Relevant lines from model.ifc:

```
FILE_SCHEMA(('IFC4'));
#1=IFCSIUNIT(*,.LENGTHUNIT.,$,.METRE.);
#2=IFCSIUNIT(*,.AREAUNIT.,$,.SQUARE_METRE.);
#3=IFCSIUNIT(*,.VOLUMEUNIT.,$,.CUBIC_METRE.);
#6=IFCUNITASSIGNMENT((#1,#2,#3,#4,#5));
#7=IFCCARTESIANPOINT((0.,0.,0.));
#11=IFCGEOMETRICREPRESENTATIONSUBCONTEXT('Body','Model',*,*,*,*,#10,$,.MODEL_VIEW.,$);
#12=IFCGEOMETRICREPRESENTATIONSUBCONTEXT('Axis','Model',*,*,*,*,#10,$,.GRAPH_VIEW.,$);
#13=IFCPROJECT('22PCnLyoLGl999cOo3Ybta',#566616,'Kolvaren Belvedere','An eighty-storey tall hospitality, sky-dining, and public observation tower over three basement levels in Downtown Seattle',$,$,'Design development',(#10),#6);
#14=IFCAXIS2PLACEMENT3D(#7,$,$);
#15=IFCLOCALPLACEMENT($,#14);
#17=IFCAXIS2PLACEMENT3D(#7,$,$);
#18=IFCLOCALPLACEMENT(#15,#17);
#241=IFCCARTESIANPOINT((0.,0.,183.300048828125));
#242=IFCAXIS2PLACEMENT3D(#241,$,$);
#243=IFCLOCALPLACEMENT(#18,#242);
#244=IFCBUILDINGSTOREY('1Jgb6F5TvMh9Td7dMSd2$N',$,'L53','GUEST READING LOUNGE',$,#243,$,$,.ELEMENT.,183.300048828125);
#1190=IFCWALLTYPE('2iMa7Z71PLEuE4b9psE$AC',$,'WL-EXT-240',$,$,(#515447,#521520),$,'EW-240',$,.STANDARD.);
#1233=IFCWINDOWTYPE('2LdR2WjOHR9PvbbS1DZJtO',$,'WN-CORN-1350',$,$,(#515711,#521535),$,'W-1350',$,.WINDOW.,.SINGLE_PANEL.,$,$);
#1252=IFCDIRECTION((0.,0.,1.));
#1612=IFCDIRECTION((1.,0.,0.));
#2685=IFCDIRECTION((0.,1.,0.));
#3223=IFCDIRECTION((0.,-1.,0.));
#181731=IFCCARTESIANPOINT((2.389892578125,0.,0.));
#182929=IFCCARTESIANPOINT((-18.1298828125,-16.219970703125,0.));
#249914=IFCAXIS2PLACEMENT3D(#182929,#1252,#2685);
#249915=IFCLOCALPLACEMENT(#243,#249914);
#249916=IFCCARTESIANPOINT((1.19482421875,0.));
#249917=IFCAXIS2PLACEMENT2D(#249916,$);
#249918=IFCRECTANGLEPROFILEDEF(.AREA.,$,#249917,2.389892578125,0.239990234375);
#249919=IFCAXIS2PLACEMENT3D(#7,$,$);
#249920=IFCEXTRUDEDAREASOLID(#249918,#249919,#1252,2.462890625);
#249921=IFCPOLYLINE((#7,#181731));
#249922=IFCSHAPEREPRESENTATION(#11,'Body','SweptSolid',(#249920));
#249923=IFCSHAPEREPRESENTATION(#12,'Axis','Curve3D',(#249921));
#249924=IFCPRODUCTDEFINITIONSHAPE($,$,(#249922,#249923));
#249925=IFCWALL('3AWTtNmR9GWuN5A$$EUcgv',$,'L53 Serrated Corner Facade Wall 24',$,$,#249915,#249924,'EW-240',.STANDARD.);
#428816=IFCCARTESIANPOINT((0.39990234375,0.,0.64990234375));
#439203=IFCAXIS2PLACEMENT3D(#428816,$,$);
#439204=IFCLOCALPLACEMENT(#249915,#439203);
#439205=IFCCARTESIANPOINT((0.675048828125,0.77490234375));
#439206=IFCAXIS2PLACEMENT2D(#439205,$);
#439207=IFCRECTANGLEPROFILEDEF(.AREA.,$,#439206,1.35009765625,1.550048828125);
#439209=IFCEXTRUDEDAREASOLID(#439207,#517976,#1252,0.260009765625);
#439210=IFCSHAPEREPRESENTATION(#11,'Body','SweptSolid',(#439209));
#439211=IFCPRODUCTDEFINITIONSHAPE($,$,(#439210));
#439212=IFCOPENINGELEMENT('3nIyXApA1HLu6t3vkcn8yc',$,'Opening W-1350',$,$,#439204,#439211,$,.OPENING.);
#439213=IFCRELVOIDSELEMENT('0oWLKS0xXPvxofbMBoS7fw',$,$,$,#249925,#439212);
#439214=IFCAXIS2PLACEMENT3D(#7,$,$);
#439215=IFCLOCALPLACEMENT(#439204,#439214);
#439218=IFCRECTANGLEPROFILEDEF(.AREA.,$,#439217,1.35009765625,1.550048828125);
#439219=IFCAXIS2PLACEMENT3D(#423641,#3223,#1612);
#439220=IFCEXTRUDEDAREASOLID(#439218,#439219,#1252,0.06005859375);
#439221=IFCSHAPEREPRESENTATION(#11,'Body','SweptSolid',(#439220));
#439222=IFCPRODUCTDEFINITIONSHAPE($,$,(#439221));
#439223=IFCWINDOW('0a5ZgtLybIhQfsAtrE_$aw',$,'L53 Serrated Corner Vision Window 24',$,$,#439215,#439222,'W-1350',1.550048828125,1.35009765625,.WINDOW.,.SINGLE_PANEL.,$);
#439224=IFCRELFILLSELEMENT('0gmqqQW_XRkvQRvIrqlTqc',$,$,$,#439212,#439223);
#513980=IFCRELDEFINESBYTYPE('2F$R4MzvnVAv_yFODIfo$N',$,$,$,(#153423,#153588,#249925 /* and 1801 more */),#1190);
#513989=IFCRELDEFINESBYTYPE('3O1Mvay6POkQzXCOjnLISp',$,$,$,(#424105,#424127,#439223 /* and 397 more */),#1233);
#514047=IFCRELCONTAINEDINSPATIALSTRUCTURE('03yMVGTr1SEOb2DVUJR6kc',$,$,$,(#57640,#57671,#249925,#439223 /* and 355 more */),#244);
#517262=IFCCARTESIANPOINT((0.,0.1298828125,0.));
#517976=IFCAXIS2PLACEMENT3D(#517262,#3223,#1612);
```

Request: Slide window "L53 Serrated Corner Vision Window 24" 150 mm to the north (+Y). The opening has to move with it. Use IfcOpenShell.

```python
import ifcopenshell
import ifcopenshell.api.geometry
import ifcopenshell.util.placement

model = ifcopenshell.open("model.ifc")

window = model.by_id(439223)
opening = window.FillsVoids[0].RelatingOpeningElement
wall = opening.VoidsElements[0].RelatingBuildingElement

wall_matrix = ifcopenshell.util.placement.get_local_placement(wall.ObjectPlacement)
shift = wall_matrix[:3, 0] * 0.15
before = ifcopenshell.util.placement.get_local_placement(window.ObjectPlacement)[:3, 3].copy()

# The window is placed relative to its opening, so it follows when the opening moves.
matrix = ifcopenshell.util.placement.get_local_placement(opening.ObjectPlacement)
matrix[:3, 3] += shift
ifcopenshell.api.geometry.edit_object_placement(
    model, product=opening, matrix=matrix, is_si=False, should_transform_children=True
)

after = ifcopenshell.util.placement.get_local_placement(window.ObjectPlacement)[:3, 3]
print("window moved by", (after - before).round(3) + 0.0)

model.write("model_rev.ifc")
```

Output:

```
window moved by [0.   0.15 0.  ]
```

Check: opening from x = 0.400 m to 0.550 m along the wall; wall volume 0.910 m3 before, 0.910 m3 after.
